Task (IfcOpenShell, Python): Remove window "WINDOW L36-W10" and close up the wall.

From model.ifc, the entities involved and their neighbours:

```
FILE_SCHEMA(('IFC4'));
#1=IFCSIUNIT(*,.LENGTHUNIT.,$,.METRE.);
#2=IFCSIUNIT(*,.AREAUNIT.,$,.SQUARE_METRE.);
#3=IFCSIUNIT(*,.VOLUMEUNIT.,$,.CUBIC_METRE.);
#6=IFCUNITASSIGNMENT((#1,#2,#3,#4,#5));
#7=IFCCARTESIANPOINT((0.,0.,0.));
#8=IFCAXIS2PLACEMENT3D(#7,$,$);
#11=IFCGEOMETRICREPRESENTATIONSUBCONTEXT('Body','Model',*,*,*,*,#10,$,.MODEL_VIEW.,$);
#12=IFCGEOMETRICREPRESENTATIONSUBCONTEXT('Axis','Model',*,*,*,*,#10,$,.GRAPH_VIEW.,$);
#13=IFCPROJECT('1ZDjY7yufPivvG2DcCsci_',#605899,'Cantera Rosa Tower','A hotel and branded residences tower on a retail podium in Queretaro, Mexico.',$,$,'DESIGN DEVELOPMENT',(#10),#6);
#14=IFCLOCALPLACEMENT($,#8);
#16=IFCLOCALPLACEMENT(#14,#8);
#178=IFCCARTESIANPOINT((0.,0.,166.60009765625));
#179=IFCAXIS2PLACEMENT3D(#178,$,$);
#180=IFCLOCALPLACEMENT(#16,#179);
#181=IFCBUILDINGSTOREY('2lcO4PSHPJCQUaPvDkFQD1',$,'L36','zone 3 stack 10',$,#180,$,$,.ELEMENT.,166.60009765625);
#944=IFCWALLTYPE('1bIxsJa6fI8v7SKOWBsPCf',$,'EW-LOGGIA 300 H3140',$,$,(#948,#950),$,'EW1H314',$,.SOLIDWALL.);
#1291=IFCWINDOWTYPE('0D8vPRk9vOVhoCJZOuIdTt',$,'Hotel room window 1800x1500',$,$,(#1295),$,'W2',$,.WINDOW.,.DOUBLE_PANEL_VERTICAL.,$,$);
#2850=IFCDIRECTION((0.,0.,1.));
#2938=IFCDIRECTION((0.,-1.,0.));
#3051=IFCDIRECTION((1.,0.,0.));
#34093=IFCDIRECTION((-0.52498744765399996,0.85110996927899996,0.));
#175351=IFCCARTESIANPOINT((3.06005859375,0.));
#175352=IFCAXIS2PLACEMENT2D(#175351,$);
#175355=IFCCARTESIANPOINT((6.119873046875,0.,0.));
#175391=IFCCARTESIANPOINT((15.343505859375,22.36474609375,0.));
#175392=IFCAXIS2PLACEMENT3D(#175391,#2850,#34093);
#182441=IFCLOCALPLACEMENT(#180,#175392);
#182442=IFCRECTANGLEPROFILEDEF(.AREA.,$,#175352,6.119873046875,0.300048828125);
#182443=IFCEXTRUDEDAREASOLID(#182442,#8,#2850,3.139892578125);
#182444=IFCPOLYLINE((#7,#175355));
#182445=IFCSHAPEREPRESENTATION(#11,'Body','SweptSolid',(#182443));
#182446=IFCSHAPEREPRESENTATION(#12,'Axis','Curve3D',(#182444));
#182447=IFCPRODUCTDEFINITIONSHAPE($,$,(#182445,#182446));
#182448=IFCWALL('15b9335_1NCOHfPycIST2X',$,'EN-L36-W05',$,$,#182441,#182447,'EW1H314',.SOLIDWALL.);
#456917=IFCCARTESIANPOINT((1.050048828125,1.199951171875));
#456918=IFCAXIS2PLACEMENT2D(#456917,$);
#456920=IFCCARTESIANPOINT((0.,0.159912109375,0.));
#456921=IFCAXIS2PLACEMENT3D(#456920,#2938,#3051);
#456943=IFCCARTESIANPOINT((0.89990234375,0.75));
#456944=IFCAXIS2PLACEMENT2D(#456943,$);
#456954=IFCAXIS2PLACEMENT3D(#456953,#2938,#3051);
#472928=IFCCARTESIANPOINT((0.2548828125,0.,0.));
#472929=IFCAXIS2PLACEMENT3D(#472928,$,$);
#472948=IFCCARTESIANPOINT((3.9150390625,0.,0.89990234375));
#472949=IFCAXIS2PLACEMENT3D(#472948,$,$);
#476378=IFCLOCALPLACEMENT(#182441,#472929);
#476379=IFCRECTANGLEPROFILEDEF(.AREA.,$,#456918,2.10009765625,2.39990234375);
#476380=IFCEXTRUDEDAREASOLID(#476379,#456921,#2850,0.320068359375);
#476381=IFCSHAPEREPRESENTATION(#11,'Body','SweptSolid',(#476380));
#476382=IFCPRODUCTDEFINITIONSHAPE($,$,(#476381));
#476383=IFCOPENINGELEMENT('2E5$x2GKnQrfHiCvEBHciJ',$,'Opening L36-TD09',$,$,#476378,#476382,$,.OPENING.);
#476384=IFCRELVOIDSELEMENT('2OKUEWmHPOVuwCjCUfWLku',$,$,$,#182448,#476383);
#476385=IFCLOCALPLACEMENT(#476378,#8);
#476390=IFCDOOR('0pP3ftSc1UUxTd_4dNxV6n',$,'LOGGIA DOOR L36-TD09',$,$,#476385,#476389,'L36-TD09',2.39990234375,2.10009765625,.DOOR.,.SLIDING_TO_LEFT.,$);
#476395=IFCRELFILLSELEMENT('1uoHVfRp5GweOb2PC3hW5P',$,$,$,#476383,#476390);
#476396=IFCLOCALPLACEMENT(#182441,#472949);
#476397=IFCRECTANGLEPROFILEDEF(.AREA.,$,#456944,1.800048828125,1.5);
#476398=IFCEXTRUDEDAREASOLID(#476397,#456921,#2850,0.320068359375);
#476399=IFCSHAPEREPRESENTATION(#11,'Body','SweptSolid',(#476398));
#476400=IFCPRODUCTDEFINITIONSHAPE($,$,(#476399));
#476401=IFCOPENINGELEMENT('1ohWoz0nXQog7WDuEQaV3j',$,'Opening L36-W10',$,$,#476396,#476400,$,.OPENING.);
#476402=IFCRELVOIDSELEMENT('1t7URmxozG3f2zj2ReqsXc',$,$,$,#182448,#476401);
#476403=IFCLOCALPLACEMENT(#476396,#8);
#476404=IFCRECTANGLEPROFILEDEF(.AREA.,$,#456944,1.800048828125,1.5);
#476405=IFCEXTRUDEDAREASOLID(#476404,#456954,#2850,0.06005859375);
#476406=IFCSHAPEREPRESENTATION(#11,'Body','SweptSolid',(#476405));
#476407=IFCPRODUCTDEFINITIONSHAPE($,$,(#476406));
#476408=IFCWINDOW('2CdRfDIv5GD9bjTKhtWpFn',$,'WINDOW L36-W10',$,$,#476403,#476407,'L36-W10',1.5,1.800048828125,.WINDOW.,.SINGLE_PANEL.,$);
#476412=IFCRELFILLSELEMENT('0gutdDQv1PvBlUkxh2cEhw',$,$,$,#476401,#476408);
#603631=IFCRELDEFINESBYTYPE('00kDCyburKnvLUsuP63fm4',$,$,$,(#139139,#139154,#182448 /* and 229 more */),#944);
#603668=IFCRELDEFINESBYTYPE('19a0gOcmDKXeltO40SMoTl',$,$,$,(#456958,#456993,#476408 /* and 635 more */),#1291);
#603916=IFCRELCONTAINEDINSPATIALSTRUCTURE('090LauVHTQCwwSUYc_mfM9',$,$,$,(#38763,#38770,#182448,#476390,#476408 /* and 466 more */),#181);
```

```python
import ifcopenshell
import ifcopenshell.api.feature
import ifcopenshell.api.root
import ifcopenshell.geom
import ifcopenshell.util.shape

model = ifcopenshell.open("model.ifc")
settings = ifcopenshell.geom.settings()


def volume(element):
    """Net volume in cubic metres, openings subtracted."""
    shape = ifcopenshell.geom.create_shape(settings, element)
    return ifcopenshell.util.shape.get_volume(shape.geometry)


window = model.by_guid("2CdRfDIv5GD9bjTKhtWpFn")
opening = window.FillsVoids[0].RelatingOpeningElement
wall = opening.VoidsElements[0].RelatingBuildingElement
before = volume(wall)

ifcopenshell.api.root.remove_product(model, product=window)
ifcopenshell.api.feature.remove_feature(model, feature=opening)

after = volume(wall)

print(f"wall volume {before:.3f} -> {after:.3f} m3")

model.write("model-out.ifc")
```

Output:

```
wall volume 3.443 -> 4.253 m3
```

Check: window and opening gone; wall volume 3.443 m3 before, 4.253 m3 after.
